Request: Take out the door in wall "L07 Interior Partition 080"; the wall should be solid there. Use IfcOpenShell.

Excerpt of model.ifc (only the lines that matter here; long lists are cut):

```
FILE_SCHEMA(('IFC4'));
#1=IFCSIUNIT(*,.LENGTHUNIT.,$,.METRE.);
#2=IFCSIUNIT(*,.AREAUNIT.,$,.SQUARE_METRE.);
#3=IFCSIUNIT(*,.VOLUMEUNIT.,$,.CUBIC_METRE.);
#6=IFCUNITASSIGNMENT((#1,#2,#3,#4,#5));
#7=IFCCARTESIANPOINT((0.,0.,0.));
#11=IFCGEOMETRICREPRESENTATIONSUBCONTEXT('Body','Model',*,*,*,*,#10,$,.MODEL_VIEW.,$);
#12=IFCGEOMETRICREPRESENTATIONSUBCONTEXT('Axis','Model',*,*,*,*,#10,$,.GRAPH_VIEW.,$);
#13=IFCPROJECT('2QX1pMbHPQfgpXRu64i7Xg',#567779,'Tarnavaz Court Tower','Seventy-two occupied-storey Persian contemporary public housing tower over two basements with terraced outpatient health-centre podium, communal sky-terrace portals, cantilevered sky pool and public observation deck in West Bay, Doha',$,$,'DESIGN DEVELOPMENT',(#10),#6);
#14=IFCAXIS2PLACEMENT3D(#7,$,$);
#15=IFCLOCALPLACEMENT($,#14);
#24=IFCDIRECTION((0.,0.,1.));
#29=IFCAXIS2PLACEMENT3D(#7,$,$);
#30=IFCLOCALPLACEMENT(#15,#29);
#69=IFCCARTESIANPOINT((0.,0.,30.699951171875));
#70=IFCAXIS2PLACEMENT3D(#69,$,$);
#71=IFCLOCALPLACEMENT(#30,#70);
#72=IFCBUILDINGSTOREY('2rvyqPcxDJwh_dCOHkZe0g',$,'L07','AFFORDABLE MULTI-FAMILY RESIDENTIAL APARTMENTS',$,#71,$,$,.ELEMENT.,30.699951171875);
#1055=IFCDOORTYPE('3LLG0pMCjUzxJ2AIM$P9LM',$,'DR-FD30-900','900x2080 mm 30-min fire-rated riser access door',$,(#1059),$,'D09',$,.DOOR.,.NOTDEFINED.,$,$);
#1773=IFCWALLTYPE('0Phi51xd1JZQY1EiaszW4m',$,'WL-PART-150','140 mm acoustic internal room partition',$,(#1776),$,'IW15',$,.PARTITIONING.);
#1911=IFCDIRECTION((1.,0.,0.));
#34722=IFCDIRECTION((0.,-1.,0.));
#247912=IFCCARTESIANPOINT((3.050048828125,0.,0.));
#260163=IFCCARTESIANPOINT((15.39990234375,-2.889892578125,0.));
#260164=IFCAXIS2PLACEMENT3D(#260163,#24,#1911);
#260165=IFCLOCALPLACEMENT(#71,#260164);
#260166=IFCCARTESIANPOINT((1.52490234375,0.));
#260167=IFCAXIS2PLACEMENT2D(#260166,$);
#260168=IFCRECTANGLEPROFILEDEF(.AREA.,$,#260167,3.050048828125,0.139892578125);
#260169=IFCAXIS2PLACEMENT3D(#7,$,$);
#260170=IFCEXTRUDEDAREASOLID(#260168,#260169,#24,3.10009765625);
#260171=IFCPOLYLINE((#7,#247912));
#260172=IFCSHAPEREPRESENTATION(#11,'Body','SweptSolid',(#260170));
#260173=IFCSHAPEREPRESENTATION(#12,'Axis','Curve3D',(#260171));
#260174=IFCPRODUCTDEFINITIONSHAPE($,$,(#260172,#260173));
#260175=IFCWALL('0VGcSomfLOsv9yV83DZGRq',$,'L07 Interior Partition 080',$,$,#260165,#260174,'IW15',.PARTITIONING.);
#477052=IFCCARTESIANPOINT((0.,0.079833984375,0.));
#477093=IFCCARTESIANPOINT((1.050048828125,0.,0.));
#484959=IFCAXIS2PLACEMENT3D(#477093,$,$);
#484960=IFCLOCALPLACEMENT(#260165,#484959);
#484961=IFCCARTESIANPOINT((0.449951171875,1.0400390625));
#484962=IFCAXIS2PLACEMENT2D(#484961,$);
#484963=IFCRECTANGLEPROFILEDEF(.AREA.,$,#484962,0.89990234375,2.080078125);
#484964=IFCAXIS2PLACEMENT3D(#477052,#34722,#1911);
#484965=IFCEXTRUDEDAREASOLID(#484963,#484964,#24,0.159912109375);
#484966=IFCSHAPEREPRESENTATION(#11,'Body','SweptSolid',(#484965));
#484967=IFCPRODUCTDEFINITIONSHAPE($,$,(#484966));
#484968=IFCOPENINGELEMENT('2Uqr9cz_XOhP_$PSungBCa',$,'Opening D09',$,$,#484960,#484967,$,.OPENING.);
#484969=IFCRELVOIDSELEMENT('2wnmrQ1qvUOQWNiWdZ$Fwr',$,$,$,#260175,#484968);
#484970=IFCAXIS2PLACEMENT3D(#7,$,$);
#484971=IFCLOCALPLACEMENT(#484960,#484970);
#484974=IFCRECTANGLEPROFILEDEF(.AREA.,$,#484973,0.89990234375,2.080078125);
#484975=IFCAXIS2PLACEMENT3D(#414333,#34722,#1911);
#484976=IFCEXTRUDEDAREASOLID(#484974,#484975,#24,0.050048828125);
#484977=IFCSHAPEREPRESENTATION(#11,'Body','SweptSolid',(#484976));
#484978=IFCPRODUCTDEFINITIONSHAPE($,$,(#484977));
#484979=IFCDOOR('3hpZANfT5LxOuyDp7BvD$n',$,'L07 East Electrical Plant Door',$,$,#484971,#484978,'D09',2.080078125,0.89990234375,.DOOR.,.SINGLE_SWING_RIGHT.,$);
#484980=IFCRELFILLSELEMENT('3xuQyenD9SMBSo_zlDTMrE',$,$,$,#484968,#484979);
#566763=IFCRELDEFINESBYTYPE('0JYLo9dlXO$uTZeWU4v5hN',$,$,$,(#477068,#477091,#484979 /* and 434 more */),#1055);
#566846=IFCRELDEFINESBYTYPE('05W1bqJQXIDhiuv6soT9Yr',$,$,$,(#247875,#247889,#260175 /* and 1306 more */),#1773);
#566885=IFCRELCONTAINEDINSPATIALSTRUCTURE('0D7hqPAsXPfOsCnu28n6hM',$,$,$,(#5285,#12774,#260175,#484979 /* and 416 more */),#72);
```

```python
import ifcopenshell
import ifcopenshell.api.feature
import ifcopenshell.api.root
import ifcopenshell.geom
import ifcopenshell.util.shape

model = ifcopenshell.open("model.ifc")
settings = ifcopenshell.geom.settings()


def volume(element):
    """Net volume in cubic metres, openings subtracted."""
    shape = ifcopenshell.geom.create_shape(settings, element)
    return ifcopenshell.util.shape.get_volume(shape.geometry)


door = model.by_guid("3hpZANfT5LxOuyDp7BvD$n")
opening = door.FillsVoids[0].RelatingOpeningElement
wall = opening.VoidsElements[0].RelatingBuildingElement
before = volume(wall)

ifcopenshell.api.root.remove_product(model, product=door)
ifcopenshell.api.feature.remove_feature(model, feature=opening)

after = volume(wall)

print(f"wall volume {before:.3f} -> {after:.3f} m3")

model.write("model_updated.ifc")
```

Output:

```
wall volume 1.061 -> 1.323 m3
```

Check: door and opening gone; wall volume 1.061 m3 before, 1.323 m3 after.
